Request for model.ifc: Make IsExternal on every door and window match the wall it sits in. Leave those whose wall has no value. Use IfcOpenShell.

First a look at what the model holds.

```python
import ifcopenshell
import ifcopenshell.util.element

model = ifcopenshell.open("model.ifc")
print(model.schema)
seen = {}
for e in model.by_type("IfcDoor") + model.by_type("IfcWindow"):
    if not e.FillsVoids:
        continue
    host = e.FillsVoids[0].RelatingOpeningElement.VoidsElements[0].RelatingBuildingElement
    own = ifcopenshell.util.element.get_pset(e, f"Pset_{e.is_a()[3:].removesuffix('StandardCase')}Common", "IsExternal")
    wall = ifcopenshell.util.element.get_pset(host, "Pset_WallCommon", "IsExternal")
    seen[e.is_a(), own, wall] = seen.get((e.is_a(), own, wall), 0) + 1
for (cls, own, wall), count in sorted(seen.items(), key=str):
    print(count, cls, "IsExternal:", own, "| host wall:", wall)
```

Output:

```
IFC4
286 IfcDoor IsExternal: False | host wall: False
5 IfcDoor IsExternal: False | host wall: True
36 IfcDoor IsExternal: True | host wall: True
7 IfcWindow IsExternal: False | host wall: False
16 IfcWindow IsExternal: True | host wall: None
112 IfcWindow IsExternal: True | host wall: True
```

```python
import ifcopenshell
import ifcopenshell.api.pset
import ifcopenshell.util.element

model = ifcopenshell.open("model.ifc")

count = 0
for ifc_class, pset_name in (("IfcDoor", "Pset_DoorCommon"), ("IfcWindow", "Pset_WindowCommon")):
    for e in model.by_type(ifc_class):
        if not e.FillsVoids:
            continue
        host = e.FillsVoids[0].RelatingOpeningElement.VoidsElements[0].RelatingBuildingElement
        external = ifcopenshell.util.element.get_pset(host, "Pset_WallCommon", "IsExternal")
        if external is None or ifcopenshell.util.element.get_pset(e, pset_name, "IsExternal") == external:
            continue
        pset = ifcopenshell.api.pset.add_pset(model, product=e, name=pset_name)
        ifcopenshell.api.pset.edit_pset(model, pset=pset, properties={"IsExternal": external})
        count += 1

print(count, "updated")

model.write("model_updated.ifc")
```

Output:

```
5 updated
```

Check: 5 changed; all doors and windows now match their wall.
